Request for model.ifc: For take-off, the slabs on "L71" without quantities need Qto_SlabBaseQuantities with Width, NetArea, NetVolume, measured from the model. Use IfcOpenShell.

First a look at what the model holds.

```python
import ifcopenshell
import ifcopenshell.util.element
import ifcopenshell.util.unit

model = ifcopenshell.open("model.ifc")
print(model.schema)
for unit_type in ("LENGTHUNIT", "AREAUNIT", "VOLUMEUNIT"):
    print(unit_type, ifcopenshell.util.unit.calculate_unit_scale(model, unit_type))
storey = next(s for s in model.by_type("IfcBuildingStorey") if s.Name == "L71")
slabs = [e for e in ifcopenshell.util.element.get_decomposition(storey) if e.is_a("IfcSlab")]
for e in sorted(slabs, key=lambda e: e.id()):
    print(e.id(), e.is_a(), e.Name, list(ifcopenshell.util.element.get_psets(e, qtos_only=True)), sep=" | ")
```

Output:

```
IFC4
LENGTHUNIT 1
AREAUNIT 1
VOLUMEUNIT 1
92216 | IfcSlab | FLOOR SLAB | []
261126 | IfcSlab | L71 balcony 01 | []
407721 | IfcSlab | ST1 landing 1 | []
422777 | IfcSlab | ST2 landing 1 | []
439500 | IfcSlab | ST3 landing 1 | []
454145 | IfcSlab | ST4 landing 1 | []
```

```python
import ifcopenshell
import ifcopenshell.api.pset
import ifcopenshell.geom
import ifcopenshell.util.element
import ifcopenshell.util.shape
import ifcopenshell.util.unit

model = ifcopenshell.open("model.ifc")
unit_scale = ifcopenshell.util.unit.calculate_unit_scale(model)
area_scale = ifcopenshell.util.unit.calculate_unit_scale(model, "AREAUNIT")
volume_scale = ifcopenshell.util.unit.calculate_unit_scale(model, "VOLUMEUNIT")
settings = ifcopenshell.geom.settings()

storey = next(s for s in model.by_type("IfcBuildingStorey") if s.Name == "L71")
slabs = [e for e in ifcopenshell.util.element.get_decomposition(storey) if e.is_a("IfcSlab")]

for e in sorted(slabs, key=lambda e: e.id()):
    if ifcopenshell.util.element.get_psets(e, qtos_only=True, should_inherit=False):
        continue
    # Geometry comes back in metres, in the element's own axes.
    shape = ifcopenshell.geom.create_shape(settings, e)
    values = {
        "Width": ifcopenshell.util.shape.get_z(shape.geometry) / unit_scale,
        "NetArea": ifcopenshell.util.shape.get_footprint_area(shape.geometry) / area_scale,
        "NetVolume": ifcopenshell.util.shape.get_volume(shape.geometry) / volume_scale,
    }
    qto = ifcopenshell.api.pset.add_qto(model, product=e, name="Qto_SlabBaseQuantities")
    ifcopenshell.api.pset.edit_qto(model, qto=qto, properties=values)
    print(e.id(), {k: round(v, 3) for k, v in values.items()})

model.write("model_edited.ifc")
```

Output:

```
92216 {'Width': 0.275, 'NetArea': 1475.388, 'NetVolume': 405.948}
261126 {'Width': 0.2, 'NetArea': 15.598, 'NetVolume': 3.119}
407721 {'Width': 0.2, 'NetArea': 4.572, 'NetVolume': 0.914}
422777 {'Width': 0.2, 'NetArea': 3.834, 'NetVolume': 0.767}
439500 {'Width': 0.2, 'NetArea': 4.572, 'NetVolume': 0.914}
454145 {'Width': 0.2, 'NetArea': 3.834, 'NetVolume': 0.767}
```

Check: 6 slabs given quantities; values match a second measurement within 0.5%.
